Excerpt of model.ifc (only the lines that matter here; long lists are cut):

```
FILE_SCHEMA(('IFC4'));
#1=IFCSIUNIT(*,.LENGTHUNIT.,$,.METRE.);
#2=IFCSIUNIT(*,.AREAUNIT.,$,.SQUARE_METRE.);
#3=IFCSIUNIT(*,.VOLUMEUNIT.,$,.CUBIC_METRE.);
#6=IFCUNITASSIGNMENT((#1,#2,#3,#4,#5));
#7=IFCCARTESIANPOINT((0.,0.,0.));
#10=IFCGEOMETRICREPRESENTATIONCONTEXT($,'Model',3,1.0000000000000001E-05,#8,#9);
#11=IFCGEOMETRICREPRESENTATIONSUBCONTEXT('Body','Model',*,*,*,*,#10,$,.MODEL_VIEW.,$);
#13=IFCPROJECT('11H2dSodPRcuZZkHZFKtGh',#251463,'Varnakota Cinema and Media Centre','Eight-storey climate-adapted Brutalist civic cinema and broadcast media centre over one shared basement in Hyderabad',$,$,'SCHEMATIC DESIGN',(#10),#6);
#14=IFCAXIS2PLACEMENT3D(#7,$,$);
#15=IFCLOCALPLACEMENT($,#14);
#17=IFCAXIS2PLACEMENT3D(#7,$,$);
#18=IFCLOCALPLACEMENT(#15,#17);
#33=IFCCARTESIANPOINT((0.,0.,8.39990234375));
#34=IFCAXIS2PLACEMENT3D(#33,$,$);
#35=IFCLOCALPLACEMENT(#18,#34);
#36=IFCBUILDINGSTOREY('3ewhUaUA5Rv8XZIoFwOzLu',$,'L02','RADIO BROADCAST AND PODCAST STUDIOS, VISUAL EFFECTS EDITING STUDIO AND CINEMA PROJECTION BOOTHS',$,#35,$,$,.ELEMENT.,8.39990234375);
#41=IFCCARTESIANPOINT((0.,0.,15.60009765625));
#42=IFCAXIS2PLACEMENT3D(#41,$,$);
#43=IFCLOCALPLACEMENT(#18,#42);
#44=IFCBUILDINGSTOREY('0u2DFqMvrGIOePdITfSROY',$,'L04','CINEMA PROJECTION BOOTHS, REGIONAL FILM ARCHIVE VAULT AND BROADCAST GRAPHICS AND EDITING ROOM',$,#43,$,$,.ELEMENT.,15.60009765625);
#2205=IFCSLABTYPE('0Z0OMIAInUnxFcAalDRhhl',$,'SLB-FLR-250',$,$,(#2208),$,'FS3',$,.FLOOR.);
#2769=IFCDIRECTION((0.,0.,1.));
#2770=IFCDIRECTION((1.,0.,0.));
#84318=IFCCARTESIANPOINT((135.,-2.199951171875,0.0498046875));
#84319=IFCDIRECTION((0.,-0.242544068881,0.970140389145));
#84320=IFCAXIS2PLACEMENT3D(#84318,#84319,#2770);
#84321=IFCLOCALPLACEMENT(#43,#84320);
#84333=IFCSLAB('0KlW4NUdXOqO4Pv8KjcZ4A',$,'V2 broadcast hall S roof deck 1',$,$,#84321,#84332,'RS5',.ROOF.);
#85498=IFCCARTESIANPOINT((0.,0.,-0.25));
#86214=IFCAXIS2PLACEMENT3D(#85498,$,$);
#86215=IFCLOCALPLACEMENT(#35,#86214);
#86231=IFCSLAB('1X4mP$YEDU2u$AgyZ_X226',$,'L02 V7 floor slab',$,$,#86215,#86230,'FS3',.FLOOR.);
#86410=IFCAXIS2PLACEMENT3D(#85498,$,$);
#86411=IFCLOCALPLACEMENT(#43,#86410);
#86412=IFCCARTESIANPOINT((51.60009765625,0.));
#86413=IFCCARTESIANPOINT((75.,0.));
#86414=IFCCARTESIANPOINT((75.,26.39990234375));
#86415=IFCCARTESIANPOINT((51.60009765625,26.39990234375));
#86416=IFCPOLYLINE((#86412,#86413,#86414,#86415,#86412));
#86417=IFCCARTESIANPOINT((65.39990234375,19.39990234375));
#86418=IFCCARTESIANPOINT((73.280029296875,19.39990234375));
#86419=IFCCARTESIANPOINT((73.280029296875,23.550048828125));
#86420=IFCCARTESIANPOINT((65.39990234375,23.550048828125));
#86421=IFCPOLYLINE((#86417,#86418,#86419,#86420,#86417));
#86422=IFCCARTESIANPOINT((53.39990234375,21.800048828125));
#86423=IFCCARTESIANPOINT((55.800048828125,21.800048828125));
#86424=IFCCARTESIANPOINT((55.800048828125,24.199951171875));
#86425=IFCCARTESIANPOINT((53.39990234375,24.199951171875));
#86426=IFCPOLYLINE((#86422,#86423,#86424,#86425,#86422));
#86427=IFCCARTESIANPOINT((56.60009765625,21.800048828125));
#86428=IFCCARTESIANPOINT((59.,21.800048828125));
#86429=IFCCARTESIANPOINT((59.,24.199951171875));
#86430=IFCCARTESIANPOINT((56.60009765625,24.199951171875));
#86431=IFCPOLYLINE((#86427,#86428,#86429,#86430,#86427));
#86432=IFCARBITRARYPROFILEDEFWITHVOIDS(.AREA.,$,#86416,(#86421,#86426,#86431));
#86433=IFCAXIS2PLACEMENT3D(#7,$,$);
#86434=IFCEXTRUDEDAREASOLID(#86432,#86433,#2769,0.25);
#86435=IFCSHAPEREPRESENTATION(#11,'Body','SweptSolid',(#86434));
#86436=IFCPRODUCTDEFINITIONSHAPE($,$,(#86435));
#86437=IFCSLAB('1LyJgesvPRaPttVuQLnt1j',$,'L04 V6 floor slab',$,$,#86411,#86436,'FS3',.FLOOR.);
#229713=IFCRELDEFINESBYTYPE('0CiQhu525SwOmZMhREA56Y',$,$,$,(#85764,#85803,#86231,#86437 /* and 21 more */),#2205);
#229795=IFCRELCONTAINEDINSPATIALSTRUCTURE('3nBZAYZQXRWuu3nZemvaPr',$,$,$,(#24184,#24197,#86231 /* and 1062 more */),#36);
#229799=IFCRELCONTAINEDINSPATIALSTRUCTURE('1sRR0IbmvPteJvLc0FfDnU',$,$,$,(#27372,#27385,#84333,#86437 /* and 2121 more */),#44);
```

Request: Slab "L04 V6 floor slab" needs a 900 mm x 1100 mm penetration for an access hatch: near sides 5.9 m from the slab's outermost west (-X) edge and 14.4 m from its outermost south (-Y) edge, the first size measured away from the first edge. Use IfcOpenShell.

```python
import numpy as np
import ifcopenshell
import ifcopenshell.api.feature
import ifcopenshell.api.geometry
import ifcopenshell.api.root
import ifcopenshell.geom
import ifcopenshell.util.placement
import ifcopenshell.util.representation
import ifcopenshell.util.shape
import ifcopenshell.util.unit

model = ifcopenshell.open("model.ifc")
unit_scale = ifcopenshell.util.unit.calculate_unit_scale(model)
settings = ifcopenshell.geom.settings()


def volume(element):
    """Net volume in cubic metres, openings subtracted."""
    shape = ifcopenshell.geom.create_shape(settings, element)
    return ifcopenshell.util.shape.get_volume(shape.geometry)


slab = model.by_guid("1LyJgesvPRaPttVuQLnt1j")
before = volume(slab)

# Extent in the slab's own axes, in metres. The edges named are its -X and -Y sides.
slab_shape = ifcopenshell.geom.create_shape(settings, slab)
vertices = ifcopenshell.util.shape.get_vertices(slab_shape.geometry)
x_min, y_min, bottom = vertices.min(axis=0)
top = vertices[:, 2].max()

opening = ifcopenshell.api.root.create_entity(model, ifc_class="IfcOpeningElement", name="Access hatch opening", predefined_type="OPENING")
context = ifcopenshell.util.representation.get_context(model, "Model", "Body", "MODEL_VIEW")
width, depth = 0.9, 1.1
outline = [(0.0, 0.0), (width, 0.0), (width, depth), (0.0, depth), (0.0, 0.0)]
# Overshoot both faces by 50 mm so the cut is clean.
shape = ifcopenshell.api.geometry.add_slab_representation(
    model, context=context, depth=top - bottom + 0.1, polyline=outline
)
ifcopenshell.api.geometry.assign_representation(model, product=opening, representation=shape)

matrix = ifcopenshell.util.placement.get_local_placement(slab.ObjectPlacement)
matrix[:, 3] = matrix @ np.append(np.array([x_min + 5.9, y_min + 14.4, bottom - 0.05]) / unit_scale, 1.0)
ifcopenshell.api.geometry.edit_object_placement(model, product=opening, matrix=matrix, is_si=False)
ifcopenshell.api.feature.add_feature(model, feature=opening, element=slab)

after = volume(slab)

print(f"slab volume {before:.3f} -> {after:.3f} m3")

model.write("model_updated.ifc")
```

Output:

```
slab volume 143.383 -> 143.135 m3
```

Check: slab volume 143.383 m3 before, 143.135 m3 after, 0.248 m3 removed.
